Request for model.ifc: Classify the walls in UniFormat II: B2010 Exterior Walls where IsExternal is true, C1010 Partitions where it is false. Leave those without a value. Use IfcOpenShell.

First a look at what the model holds.

```python
import ifcopenshell
import ifcopenshell.util.element

model = ifcopenshell.open("model.ifc")
print(model.schema)
print("classifications:", [c.Name for c in model.by_type("IfcClassification")])
values = [ifcopenshell.util.element.get_pset(e, "Pset_WallCommon", "IsExternal") for e in model.by_type("IfcWall")]
for value in (True, False, None):
    print("IsExternal", value, values.count(value))
```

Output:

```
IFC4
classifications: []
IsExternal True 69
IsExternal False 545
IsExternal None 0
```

```python
import ifcopenshell
import ifcopenshell.api.classification
import ifcopenshell.util.element

model = ifcopenshell.open("model.ifc")

system = ifcopenshell.api.classification.add_classification(model, classification="UniFormat II")

walls = model.by_type("IfcWall")
external = {e: ifcopenshell.util.element.get_pset(e, "Pset_WallCommon", "IsExternal") for e in walls}
for flag, code, name in ((True, "B2010", "Exterior Walls"), (False, "C1010", "Partitions")):
    products = [e for e in walls if external[e] is flag]
    ifcopenshell.api.classification.add_reference(
        model, products=products, classification=system, identification=code, name=name
    )
    print(code, len(products))

model.write("model_updated.ifc")
```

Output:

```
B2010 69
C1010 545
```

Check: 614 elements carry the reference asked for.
